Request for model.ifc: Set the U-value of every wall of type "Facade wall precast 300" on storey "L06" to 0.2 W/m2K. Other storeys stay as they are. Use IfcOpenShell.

First a look at what the model holds.

```python
import ifcopenshell
import ifcopenshell.util.element

model = ifcopenshell.open("model.ifc")
print(model.schema)
storey = next(s for s in model.by_type("IfcBuildingStorey") if s.Name == "L06")
walls = [e for e in ifcopenshell.util.element.get_decomposition(storey) if e.is_a("IfcWall")]
seen = {}
for e in walls:
    element_type = ifcopenshell.util.element.get_type(e)
    key = (element_type.Name if element_type != e and element_type else None, ifcopenshell.util.element.get_pset(e, "Pset_WallCommon", "ThermalTransmittance"))
    seen[key] = seen.get(key, 0) + 1
for (name, value), count in sorted(seen.items(), key=str):
    print(count, "x", name, "|", value)
```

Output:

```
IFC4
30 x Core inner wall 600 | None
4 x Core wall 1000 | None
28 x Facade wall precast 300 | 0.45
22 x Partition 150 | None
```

```python
import ifcopenshell
import ifcopenshell.api.pset
import ifcopenshell.util.element

model = ifcopenshell.open("model.ifc")

storey = next(s for s in model.by_type("IfcBuildingStorey") if s.Name == "L06")
walls = [e for e in ifcopenshell.util.element.get_decomposition(storey) if e.is_a("IfcWall")]

count = 0
for e in walls:
    element_type = ifcopenshell.util.element.get_type(e)
    if element_type in (None, e) or element_type.Name != "Facade wall precast 300":
        continue
    # add_pset returns the element's existing set when there is one.
    pset = ifcopenshell.api.pset.add_pset(model, product=e, name="Pset_WallCommon")
    ifcopenshell.api.pset.edit_pset(model, pset=pset, properties={"ThermalTransmittance": 0.2})
    count += 1

print(count, "walls updated")

model.write("model_rev.ifc")
```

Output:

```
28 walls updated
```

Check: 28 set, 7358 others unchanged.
